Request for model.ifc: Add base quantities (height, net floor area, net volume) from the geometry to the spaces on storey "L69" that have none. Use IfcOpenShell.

First a look at what the model holds.

```python
import ifcopenshell
import ifcopenshell.util.element
import ifcopenshell.util.unit

model = ifcopenshell.open("model.ifc")
print(model.schema)
for unit_type in ("LENGTHUNIT", "AREAUNIT", "VOLUMEUNIT"):
    print(unit_type, ifcopenshell.util.unit.calculate_unit_scale(model, unit_type))
storey = next(s for s in model.by_type("IfcBuildingStorey") if s.Name == "L69")
spaces = [e for e in ifcopenshell.util.element.get_decomposition(storey) if e.is_a("IfcSpace")]
for e in sorted(spaces, key=lambda e: e.id()):
    print(e.id(), e.is_a(), e.Name, list(ifcopenshell.util.element.get_psets(e, qtos_only=True)), sep=" | ")
```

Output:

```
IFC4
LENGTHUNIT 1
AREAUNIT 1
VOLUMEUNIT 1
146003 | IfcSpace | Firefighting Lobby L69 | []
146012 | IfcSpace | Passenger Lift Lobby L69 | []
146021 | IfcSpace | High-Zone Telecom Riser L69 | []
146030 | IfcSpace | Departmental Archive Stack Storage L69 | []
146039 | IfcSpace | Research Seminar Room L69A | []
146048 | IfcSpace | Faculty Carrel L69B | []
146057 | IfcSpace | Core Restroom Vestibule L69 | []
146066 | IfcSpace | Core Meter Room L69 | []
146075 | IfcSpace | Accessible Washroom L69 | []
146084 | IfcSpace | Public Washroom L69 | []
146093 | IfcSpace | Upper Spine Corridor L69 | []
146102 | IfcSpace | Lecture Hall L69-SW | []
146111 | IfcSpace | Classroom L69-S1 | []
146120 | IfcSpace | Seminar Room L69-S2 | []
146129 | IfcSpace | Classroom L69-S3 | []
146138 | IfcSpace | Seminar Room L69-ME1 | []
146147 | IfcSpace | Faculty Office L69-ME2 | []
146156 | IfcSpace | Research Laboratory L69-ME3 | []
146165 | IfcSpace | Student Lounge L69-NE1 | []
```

```python
import ifcopenshell
import ifcopenshell.api.pset
import ifcopenshell.geom
import ifcopenshell.util.element
import ifcopenshell.util.shape
import ifcopenshell.util.unit

model = ifcopenshell.open("model.ifc")
unit_scale = ifcopenshell.util.unit.calculate_unit_scale(model)
area_scale = ifcopenshell.util.unit.calculate_unit_scale(model, "AREAUNIT")
volume_scale = ifcopenshell.util.unit.calculate_unit_scale(model, "VOLUMEUNIT")
settings = ifcopenshell.geom.settings()

storey = next(s for s in model.by_type("IfcBuildingStorey") if s.Name == "L69")
spaces = [e for e in ifcopenshell.util.element.get_decomposition(storey) if e.is_a("IfcSpace")]

for e in sorted(spaces, key=lambda e: e.id()):
    if ifcopenshell.util.element.get_psets(e, qtos_only=True, should_inherit=False):
        continue
    # Geometry comes back in metres, in the element's own axes.
    shape = ifcopenshell.geom.create_shape(settings, e)
    values = {
        "Height": ifcopenshell.util.shape.get_z(shape.geometry) / unit_scale,
        "NetFloorArea": ifcopenshell.util.shape.get_footprint_area(shape.geometry) / area_scale,
        "NetVolume": ifcopenshell.util.shape.get_volume(shape.geometry) / volume_scale,
    }
    qto = ifcopenshell.api.pset.add_qto(model, product=e, name="Qto_SpaceBaseQuantities")
    ifcopenshell.api.pset.edit_qto(model, qto=qto, properties=values)
    print(e.id(), {k: round(v, 3) for k, v in values.items()})

model.write("model_updated.ifc")
```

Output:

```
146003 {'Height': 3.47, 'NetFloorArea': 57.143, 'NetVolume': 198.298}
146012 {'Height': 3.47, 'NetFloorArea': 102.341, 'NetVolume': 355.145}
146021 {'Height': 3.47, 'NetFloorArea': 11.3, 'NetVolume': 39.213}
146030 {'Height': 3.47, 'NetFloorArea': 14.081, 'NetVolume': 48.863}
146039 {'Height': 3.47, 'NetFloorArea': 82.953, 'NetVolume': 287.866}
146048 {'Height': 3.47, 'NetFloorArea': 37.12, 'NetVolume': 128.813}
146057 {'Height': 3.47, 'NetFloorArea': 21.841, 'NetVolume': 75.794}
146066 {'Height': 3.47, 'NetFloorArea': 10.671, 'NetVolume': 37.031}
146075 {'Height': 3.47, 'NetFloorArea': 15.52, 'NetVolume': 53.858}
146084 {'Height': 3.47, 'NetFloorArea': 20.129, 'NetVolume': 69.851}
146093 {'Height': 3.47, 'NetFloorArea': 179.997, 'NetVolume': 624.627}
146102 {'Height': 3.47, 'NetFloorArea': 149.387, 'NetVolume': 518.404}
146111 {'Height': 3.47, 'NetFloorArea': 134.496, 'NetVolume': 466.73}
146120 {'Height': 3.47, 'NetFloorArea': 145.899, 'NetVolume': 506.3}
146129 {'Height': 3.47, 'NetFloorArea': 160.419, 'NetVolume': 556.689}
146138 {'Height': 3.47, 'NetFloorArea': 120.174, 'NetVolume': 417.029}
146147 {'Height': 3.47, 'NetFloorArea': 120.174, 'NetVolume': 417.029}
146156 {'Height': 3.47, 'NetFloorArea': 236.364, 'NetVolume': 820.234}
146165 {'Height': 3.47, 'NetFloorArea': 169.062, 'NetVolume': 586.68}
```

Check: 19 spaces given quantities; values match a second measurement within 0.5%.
